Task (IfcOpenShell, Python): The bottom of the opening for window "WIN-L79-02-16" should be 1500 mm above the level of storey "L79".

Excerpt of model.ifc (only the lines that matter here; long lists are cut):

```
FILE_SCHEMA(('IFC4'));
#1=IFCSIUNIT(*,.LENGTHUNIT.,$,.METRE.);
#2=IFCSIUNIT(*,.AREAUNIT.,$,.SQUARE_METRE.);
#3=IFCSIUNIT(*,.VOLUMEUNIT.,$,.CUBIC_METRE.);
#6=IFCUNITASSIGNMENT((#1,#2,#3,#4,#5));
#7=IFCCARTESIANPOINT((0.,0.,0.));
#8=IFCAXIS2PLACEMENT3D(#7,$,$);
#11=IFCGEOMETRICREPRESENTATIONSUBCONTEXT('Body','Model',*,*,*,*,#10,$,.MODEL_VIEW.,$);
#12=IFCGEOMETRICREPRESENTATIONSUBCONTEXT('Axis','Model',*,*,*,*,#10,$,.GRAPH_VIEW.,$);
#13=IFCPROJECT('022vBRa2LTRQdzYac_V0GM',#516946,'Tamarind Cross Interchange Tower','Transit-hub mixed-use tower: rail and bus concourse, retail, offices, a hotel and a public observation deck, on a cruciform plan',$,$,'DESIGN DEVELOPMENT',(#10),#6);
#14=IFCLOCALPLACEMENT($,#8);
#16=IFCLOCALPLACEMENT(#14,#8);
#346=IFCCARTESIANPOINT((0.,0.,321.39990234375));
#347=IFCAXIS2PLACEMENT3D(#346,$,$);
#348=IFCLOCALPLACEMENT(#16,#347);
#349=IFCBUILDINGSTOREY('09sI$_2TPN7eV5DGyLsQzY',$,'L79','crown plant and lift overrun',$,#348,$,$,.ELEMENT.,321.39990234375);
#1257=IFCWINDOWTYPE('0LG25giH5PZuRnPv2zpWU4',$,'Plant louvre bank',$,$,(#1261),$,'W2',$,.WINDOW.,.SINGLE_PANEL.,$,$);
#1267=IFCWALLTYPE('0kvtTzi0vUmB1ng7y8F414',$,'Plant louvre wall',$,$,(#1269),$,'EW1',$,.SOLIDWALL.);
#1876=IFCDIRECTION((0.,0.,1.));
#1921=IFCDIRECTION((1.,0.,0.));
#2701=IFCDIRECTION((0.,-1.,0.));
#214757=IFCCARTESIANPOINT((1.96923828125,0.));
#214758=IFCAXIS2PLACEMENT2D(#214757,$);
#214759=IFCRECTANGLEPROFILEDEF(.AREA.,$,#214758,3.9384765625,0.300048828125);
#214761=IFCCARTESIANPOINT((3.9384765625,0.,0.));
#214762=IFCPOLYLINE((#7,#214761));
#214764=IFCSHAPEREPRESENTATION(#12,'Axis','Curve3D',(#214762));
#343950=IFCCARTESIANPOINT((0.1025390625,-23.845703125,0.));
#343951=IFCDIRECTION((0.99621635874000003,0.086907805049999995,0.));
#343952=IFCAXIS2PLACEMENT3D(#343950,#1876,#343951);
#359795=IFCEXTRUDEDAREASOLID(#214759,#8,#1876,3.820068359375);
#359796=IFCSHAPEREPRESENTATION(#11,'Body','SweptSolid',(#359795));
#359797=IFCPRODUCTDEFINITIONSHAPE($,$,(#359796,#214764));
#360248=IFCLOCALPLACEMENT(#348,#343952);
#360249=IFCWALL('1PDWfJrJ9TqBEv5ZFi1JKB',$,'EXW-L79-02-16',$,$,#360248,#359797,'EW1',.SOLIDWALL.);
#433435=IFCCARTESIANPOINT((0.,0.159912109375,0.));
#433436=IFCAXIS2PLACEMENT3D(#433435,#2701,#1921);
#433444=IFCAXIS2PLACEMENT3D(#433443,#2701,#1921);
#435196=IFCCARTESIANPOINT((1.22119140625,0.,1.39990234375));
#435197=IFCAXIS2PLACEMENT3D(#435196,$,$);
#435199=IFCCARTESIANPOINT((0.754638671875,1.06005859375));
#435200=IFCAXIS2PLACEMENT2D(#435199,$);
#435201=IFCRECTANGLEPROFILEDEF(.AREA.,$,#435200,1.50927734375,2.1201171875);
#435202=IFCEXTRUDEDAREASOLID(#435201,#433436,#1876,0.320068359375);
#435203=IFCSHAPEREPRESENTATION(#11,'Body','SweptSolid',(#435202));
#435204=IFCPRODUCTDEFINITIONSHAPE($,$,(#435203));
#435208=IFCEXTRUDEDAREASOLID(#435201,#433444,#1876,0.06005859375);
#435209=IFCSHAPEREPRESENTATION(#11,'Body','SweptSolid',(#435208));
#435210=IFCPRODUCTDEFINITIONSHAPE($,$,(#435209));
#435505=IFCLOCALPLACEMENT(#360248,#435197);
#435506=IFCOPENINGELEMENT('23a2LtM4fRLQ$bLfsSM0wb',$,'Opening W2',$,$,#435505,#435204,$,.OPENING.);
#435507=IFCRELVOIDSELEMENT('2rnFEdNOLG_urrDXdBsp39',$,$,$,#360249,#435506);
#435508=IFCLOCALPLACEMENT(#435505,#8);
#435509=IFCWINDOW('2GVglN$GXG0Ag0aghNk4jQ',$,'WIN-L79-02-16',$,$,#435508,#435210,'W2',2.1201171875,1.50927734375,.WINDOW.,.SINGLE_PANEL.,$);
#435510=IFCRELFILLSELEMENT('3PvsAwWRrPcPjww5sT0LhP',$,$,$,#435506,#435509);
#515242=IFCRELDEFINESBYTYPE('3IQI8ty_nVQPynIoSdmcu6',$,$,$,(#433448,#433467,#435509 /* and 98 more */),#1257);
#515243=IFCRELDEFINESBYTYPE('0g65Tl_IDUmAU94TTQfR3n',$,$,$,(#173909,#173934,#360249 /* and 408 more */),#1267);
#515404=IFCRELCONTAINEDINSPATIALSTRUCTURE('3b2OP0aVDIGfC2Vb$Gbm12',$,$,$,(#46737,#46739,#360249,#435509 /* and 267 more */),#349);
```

```python
import numpy as np
import ifcopenshell
import ifcopenshell.api.geometry
import ifcopenshell.geom
import ifcopenshell.util.element
import ifcopenshell.util.placement
import ifcopenshell.util.shape
import ifcopenshell.util.unit

model = ifcopenshell.open("model.ifc")
unit_scale = ifcopenshell.util.unit.calculate_unit_scale(model)

window = model.by_guid("2GVglN$GXG0Ag0aghNk4jQ")
opening = window.FillsVoids[0].RelatingOpeningElement
storey = ifcopenshell.util.element.get_container(window, ifc_class="IfcBuildingStorey")
level = ifcopenshell.util.placement.get_local_placement(storey.ObjectPlacement)[2, 3]

# The opening's origin need not be at the sill, so measure its lowest point.
shape = ifcopenshell.geom.create_shape(ifcopenshell.geom.settings(), opening)
bottom = ifcopenshell.util.shape.get_shape_bottom_elevation(shape, shape.geometry) / unit_scale
dz = level + 1.5 / unit_scale - bottom

shift = np.array([0.0, 0.0, dz])
# The window is placed relative to its opening, so it follows when the opening moves.
matrix = ifcopenshell.util.placement.get_local_placement(opening.ObjectPlacement)
matrix[:3, 3] += shift
ifcopenshell.api.geometry.edit_object_placement(
    model, product=opening, matrix=matrix, is_si=False, should_transform_children=True
)

print(f"moved by {dz * unit_scale:+.3f} m")

model.write("model_rev.ifc")
```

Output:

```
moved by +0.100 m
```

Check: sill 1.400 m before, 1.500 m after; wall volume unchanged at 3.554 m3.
